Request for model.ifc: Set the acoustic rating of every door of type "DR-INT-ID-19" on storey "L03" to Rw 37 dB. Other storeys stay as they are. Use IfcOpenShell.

First a look at what the model holds.

```python
import ifcopenshell
import ifcopenshell.util.element

model = ifcopenshell.open("model.ifc")
print(model.schema)
storey = next(s for s in model.by_type("IfcBuildingStorey") if s.Name == "L03")
doors = [e for e in ifcopenshell.util.element.get_decomposition(storey) if e.is_a("IfcDoor")]
seen = {}
for e in doors:
    element_type = ifcopenshell.util.element.get_type(e)
    key = (element_type.Name if element_type != e and element_type else None, ifcopenshell.util.element.get_pset(e, "Pset_DoorCommon", "AcousticRating"))
    seen[key] = seen.get(key, 0) + 1
for (name, value), count in sorted(seen.items(), key=str):
    print(count, "x", name, "|", value)
```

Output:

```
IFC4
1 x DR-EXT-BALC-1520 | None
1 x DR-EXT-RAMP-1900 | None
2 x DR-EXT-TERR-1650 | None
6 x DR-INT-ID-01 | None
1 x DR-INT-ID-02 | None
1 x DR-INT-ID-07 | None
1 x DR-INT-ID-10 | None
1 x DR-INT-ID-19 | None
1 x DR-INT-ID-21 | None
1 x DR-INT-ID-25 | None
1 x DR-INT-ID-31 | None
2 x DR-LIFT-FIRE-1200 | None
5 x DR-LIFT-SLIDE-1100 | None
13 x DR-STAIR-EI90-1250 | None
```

```python
import ifcopenshell
import ifcopenshell.api.pset
import ifcopenshell.util.element

model = ifcopenshell.open("model.ifc")

storey = next(s for s in model.by_type("IfcBuildingStorey") if s.Name == "L03")
doors = [e for e in ifcopenshell.util.element.get_decomposition(storey) if e.is_a("IfcDoor")]

count = 0
for e in doors:
    element_type = ifcopenshell.util.element.get_type(e)
    if element_type in (None, e) or element_type.Name != "DR-INT-ID-19":
        continue
    # add_pset returns the element's existing set when there is one.
    pset = ifcopenshell.api.pset.add_pset(model, product=e, name="Pset_DoorCommon")
    ifcopenshell.api.pset.edit_pset(model, pset=pset, properties={"AcousticRating": "Rw 37 dB"})
    count += 1

print(count, "doors updated")

model.write("model_updated.ifc")
```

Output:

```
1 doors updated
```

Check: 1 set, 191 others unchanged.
